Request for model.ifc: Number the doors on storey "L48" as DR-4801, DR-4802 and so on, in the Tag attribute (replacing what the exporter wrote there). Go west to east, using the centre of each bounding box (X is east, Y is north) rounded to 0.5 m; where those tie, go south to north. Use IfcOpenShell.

First a look at what the model holds.

```python
import ifcopenshell
import ifcopenshell.util.element
import ifcopenshell.util.placement

model = ifcopenshell.open("model.ifc")
print(model.schema)
storey = next(s for s in model.by_type("IfcBuildingStorey") if s.Name == "L48")
doors = [e for e in ifcopenshell.util.element.get_decomposition(storey) if e.is_a("IfcDoor")]
for e in sorted(doors, key=lambda e: e.id()):
    origin = ifcopenshell.util.placement.get_local_placement(e.ObjectPlacement)[:3, 3]
    print(e.id(), e.Tag, e.Name, origin.round(2) + 0.0, sep=" | ")
```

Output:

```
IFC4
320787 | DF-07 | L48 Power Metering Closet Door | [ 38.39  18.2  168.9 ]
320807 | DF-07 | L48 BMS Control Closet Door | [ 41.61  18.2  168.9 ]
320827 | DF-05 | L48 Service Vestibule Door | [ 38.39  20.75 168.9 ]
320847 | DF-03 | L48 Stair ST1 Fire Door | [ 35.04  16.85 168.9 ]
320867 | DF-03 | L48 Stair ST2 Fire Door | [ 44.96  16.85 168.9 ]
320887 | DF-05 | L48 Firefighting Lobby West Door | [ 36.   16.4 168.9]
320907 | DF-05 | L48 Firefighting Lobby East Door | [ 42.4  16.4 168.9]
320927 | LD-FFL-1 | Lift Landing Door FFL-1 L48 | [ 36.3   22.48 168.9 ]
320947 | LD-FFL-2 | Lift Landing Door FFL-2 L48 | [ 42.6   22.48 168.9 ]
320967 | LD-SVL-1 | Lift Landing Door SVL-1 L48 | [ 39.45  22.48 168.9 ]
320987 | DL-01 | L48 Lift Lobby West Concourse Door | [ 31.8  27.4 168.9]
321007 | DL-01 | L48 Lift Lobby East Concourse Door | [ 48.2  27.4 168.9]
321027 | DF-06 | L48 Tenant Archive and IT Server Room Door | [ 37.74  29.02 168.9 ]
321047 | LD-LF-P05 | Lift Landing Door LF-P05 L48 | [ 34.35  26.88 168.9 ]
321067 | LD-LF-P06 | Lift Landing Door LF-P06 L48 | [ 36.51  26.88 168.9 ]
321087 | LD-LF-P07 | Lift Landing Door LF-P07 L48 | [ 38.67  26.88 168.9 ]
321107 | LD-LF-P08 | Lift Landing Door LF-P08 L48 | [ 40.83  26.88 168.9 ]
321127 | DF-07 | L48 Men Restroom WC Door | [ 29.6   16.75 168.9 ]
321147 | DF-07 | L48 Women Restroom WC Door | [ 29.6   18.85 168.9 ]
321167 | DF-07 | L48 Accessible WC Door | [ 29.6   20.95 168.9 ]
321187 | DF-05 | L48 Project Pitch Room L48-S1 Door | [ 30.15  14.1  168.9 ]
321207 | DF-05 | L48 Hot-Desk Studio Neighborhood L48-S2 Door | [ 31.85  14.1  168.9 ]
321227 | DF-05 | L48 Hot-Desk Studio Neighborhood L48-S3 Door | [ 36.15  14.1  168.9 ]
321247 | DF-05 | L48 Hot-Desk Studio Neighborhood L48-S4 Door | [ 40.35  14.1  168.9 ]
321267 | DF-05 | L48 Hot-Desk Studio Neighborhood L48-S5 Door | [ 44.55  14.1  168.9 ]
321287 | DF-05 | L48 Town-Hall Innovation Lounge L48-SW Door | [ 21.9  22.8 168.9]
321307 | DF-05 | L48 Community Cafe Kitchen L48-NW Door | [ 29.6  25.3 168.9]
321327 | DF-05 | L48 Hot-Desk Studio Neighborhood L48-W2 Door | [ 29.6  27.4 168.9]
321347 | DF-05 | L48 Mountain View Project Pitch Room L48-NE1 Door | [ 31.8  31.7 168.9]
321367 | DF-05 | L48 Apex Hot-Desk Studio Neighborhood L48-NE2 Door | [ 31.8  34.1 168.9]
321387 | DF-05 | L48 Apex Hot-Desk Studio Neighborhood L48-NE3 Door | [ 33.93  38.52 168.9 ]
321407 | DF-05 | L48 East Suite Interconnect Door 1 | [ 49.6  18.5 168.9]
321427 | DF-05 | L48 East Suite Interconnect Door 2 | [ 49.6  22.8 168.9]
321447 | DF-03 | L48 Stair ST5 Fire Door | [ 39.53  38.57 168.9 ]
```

```python
import ifcopenshell
import ifcopenshell.geom
import ifcopenshell.util.element
import ifcopenshell.util.shape

model = ifcopenshell.open("model.ifc")
settings = ifcopenshell.geom.settings()
settings.set("use-world-coords", True)


def centre(element):
    shape = ifcopenshell.geom.create_shape(settings, element)
    return ifcopenshell.util.shape.get_bbox_centroid(shape.geometry)


storey = next(s for s in model.by_type("IfcBuildingStorey") if s.Name == "L48")
doors = [e for e in ifcopenshell.util.element.get_decomposition(storey) if e.is_a("IfcDoor")]

# Insertion points can sit at a corner or the storey origin, so sort by the geometry (in metres).
centres = {e: centre(e) for e in doors}
doors.sort(key=lambda e: (round(centres[e][0] / 0.5), centres[e][1]))

for i, e in enumerate(doors, start=1):
    number = f"DR-48{i:02d}"
    e.Tag = number
    print(e.id(), number)

model.write("model_updated.ifc")
```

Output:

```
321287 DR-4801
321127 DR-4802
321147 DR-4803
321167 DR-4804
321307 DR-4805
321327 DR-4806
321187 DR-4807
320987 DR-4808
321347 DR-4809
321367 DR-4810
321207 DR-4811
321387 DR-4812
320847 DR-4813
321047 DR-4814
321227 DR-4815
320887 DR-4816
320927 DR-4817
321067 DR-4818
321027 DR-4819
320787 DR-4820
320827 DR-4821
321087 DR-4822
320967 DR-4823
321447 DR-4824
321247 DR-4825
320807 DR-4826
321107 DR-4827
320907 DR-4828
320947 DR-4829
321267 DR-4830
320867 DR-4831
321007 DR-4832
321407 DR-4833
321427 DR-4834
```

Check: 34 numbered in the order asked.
